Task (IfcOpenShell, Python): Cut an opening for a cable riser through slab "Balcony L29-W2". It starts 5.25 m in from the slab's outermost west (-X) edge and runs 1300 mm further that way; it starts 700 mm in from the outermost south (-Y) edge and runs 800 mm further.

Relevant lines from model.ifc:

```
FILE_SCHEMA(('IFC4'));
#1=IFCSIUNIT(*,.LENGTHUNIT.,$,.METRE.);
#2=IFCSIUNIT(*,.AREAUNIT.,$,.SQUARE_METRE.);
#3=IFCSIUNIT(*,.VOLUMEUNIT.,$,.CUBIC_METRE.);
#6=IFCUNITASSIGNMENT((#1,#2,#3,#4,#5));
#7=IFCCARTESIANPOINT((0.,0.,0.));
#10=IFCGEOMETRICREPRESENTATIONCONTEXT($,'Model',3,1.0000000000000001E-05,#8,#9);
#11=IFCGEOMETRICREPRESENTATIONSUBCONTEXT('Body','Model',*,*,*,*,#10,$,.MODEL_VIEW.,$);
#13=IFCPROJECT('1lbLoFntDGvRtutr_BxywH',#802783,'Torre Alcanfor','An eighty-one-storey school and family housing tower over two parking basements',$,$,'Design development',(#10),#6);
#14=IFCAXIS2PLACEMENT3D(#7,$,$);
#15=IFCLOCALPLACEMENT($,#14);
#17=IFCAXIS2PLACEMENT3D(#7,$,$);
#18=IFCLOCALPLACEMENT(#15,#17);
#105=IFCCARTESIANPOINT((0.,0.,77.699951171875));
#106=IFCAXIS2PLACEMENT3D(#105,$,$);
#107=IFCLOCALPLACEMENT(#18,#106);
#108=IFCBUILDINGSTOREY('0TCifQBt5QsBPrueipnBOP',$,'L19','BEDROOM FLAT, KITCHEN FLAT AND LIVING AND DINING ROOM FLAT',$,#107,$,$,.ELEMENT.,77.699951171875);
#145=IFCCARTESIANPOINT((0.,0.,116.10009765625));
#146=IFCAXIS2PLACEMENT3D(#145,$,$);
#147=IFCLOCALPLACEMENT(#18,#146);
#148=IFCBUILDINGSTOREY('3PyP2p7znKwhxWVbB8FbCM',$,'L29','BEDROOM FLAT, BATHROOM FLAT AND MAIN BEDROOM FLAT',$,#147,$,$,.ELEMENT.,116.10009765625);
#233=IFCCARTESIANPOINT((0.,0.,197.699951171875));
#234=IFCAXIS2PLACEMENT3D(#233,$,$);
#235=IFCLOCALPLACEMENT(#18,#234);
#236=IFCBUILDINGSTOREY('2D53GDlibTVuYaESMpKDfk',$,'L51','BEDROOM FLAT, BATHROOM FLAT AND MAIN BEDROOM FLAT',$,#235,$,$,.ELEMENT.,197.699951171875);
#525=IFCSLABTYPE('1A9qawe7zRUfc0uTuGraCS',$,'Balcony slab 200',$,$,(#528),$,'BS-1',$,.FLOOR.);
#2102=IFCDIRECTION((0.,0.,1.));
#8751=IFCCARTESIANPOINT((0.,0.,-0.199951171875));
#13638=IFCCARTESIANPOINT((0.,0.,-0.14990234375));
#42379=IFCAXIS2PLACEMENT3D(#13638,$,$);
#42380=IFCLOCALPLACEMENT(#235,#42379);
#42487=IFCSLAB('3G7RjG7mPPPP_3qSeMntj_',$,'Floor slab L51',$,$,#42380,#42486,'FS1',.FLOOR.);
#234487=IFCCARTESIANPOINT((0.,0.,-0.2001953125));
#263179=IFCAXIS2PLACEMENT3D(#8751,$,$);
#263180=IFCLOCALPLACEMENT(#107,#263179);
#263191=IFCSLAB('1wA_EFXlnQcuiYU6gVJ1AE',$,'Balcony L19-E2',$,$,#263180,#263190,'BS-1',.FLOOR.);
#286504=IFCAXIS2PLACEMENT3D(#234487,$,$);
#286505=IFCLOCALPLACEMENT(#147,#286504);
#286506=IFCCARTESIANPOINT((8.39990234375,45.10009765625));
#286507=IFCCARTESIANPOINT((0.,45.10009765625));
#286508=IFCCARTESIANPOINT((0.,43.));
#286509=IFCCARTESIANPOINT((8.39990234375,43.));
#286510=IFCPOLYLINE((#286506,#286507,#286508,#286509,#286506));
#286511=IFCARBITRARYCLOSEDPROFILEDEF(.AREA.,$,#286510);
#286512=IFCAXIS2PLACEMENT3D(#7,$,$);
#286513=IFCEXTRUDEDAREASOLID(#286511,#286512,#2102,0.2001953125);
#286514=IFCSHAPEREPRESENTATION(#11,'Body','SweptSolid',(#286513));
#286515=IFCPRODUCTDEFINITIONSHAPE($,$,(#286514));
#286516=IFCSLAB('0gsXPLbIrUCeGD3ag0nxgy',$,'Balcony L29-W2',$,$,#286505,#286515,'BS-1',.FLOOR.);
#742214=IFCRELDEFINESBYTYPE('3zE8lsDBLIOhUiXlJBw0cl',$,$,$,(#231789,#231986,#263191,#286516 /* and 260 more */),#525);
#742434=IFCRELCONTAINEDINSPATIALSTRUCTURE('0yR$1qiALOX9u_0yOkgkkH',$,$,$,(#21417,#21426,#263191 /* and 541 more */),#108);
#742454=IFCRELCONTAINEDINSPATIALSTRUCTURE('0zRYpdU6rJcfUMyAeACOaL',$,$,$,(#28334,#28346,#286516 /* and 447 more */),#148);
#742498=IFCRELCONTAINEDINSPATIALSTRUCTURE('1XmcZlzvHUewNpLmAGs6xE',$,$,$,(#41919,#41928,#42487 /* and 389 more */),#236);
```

```python
import numpy as np
import ifcopenshell
import ifcopenshell.api.feature
import ifcopenshell.api.geometry
import ifcopenshell.api.root
import ifcopenshell.geom
import ifcopenshell.util.placement
import ifcopenshell.util.representation
import ifcopenshell.util.shape
import ifcopenshell.util.unit

model = ifcopenshell.open("model.ifc")
unit_scale = ifcopenshell.util.unit.calculate_unit_scale(model)
settings = ifcopenshell.geom.settings()


def volume(element):
    """Net volume in cubic metres, openings subtracted."""
    shape = ifcopenshell.geom.create_shape(settings, element)
    return ifcopenshell.util.shape.get_volume(shape.geometry)


slab = model.by_id(286516)
before = volume(slab)

# Extent in the slab's own axes, in metres. The edges named are its -X and -Y sides.
slab_shape = ifcopenshell.geom.create_shape(settings, slab)
vertices = ifcopenshell.util.shape.get_vertices(slab_shape.geometry)
x_min, y_min, bottom = vertices.min(axis=0)
top = vertices[:, 2].max()

opening = ifcopenshell.api.root.create_entity(model, ifc_class="IfcOpeningElement", name="Cable riser opening", predefined_type="OPENING")
context = ifcopenshell.util.representation.get_context(model, "Model", "Body", "MODEL_VIEW")
width, depth = 1.3, 0.8
outline = [(0.0, 0.0), (width, 0.0), (width, depth), (0.0, depth), (0.0, 0.0)]
# Overshoot both faces by 50 mm so the cut is clean.
shape = ifcopenshell.api.geometry.add_slab_representation(
    model, context=context, depth=top - bottom + 0.1, polyline=outline
)
ifcopenshell.api.geometry.assign_representation(model, product=opening, representation=shape)

matrix = ifcopenshell.util.placement.get_local_placement(slab.ObjectPlacement)
matrix[:, 3] = matrix @ np.append(np.array([x_min + 5.25, y_min + 0.7, bottom - 0.05]) / unit_scale, 1.0)
ifcopenshell.api.geometry.edit_object_placement(model, product=opening, matrix=matrix, is_si=False)
ifcopenshell.api.feature.add_feature(model, feature=opening, element=slab)

after = volume(slab)

print(f"slab volume {before:.3f} -> {after:.3f} m3")

model.write("model_v2.ifc")
```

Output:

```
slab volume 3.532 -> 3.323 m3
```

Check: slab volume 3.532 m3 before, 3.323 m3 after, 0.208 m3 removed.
